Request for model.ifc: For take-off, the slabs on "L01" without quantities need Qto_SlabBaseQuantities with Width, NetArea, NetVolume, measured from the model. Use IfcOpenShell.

First a look at what the model holds.

```python
import ifcopenshell
import ifcopenshell.util.element
import ifcopenshell.util.unit

model = ifcopenshell.open("model.ifc")
print(model.schema)
for unit_type in ("LENGTHUNIT", "AREAUNIT", "VOLUMEUNIT"):
    print(unit_type, ifcopenshell.util.unit.calculate_unit_scale(model, unit_type))
storey = next(s for s in model.by_type("IfcBuildingStorey") if s.Name == "L01")
slabs = [e for e in ifcopenshell.util.element.get_decomposition(storey) if e.is_a("IfcSlab")]
for e in sorted(slabs, key=lambda e: e.id()):
    print(e.id(), e.is_a(), e.Name, list(ifcopenshell.util.element.get_psets(e, qtos_only=True)), sep=" | ")
```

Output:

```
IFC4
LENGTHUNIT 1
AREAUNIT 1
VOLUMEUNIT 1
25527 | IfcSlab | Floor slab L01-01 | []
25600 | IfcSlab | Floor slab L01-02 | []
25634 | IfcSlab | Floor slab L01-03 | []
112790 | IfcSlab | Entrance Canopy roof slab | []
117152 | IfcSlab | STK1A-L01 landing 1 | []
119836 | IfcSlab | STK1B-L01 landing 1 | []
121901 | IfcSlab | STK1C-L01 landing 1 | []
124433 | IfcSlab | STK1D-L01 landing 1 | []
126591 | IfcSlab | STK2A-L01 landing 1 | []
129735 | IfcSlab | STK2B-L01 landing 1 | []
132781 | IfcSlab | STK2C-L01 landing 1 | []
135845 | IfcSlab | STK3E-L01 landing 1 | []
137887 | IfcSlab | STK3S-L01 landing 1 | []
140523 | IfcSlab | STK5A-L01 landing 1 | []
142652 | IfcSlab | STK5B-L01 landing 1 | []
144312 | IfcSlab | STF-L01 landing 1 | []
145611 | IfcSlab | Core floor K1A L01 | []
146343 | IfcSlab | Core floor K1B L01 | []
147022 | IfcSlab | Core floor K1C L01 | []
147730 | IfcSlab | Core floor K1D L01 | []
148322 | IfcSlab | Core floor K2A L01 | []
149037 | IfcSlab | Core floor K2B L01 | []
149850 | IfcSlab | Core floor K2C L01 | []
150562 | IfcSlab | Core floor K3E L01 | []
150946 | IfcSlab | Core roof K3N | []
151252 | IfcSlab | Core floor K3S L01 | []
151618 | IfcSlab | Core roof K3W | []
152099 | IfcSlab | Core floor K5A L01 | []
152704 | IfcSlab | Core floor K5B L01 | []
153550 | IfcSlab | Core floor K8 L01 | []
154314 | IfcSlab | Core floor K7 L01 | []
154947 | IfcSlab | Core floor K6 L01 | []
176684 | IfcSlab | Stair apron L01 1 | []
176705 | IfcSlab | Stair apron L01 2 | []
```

```python
import ifcopenshell
import ifcopenshell.api.pset
import ifcopenshell.geom
import ifcopenshell.util.element
import ifcopenshell.util.shape
import ifcopenshell.util.unit

model = ifcopenshell.open("model.ifc")
unit_scale = ifcopenshell.util.unit.calculate_unit_scale(model)
area_scale = ifcopenshell.util.unit.calculate_unit_scale(model, "AREAUNIT")
volume_scale = ifcopenshell.util.unit.calculate_unit_scale(model, "VOLUMEUNIT")
settings = ifcopenshell.geom.settings()

storey = next(s for s in model.by_type("IfcBuildingStorey") if s.Name == "L01")
slabs = [e for e in ifcopenshell.util.element.get_decomposition(storey) if e.is_a("IfcSlab")]

for e in sorted(slabs, key=lambda e: e.id()):
    if ifcopenshell.util.element.get_psets(e, qtos_only=True, should_inherit=False):
        continue
    # Geometry comes back in metres, in the element's own axes.
    shape = ifcopenshell.geom.create_shape(settings, e)
    values = {
        "Width": ifcopenshell.util.shape.get_z(shape.geometry) / unit_scale,
        "NetArea": ifcopenshell.util.shape.get_footprint_area(shape.geometry) / area_scale,
        "NetVolume": ifcopenshell.util.shape.get_volume(shape.geometry) / volume_scale,
    }
    qto = ifcopenshell.api.pset.add_qto(model, product=e, name="Qto_SlabBaseQuantities")
    ifcopenshell.api.pset.edit_qto(model, qto=qto, properties=values)
    print(e.id(), {k: round(v, 3) for k, v in values.items()})

model.write("model_v2.ifc")
```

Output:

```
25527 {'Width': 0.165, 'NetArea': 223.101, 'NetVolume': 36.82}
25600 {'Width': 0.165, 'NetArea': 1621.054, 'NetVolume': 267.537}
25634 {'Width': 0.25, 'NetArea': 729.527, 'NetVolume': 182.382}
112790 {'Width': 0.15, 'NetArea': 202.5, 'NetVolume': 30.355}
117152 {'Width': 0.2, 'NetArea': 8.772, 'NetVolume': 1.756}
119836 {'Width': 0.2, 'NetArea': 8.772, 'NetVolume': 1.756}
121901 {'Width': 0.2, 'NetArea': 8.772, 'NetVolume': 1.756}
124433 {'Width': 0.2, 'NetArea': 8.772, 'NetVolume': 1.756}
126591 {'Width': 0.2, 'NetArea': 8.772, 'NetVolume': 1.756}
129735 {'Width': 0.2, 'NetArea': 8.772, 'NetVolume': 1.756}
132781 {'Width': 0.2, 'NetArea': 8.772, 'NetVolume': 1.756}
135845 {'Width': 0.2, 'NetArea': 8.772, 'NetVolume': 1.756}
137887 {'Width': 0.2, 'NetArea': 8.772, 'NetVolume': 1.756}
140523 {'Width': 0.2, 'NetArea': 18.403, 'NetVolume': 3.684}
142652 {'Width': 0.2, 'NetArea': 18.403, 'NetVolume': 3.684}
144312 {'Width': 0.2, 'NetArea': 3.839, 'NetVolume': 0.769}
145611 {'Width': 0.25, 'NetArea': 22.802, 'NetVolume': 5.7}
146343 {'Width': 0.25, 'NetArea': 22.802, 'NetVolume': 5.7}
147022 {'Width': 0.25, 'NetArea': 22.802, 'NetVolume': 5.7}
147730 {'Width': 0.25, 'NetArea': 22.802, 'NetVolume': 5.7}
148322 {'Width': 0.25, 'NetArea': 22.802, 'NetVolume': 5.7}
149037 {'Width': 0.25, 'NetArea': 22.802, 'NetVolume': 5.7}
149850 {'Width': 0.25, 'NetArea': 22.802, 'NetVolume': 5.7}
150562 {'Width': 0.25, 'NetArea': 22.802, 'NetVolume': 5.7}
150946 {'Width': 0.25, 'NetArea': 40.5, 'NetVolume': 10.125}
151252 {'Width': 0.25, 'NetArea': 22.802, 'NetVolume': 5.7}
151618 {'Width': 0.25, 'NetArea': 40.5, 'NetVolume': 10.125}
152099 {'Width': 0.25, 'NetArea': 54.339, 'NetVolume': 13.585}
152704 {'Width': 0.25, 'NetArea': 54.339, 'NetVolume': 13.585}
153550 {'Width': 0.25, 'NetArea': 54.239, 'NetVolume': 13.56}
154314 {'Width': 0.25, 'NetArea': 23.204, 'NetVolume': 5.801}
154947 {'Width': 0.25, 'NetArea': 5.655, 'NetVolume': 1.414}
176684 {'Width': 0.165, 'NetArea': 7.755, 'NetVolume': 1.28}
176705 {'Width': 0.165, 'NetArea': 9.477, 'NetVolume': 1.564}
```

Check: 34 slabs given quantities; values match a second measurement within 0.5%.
